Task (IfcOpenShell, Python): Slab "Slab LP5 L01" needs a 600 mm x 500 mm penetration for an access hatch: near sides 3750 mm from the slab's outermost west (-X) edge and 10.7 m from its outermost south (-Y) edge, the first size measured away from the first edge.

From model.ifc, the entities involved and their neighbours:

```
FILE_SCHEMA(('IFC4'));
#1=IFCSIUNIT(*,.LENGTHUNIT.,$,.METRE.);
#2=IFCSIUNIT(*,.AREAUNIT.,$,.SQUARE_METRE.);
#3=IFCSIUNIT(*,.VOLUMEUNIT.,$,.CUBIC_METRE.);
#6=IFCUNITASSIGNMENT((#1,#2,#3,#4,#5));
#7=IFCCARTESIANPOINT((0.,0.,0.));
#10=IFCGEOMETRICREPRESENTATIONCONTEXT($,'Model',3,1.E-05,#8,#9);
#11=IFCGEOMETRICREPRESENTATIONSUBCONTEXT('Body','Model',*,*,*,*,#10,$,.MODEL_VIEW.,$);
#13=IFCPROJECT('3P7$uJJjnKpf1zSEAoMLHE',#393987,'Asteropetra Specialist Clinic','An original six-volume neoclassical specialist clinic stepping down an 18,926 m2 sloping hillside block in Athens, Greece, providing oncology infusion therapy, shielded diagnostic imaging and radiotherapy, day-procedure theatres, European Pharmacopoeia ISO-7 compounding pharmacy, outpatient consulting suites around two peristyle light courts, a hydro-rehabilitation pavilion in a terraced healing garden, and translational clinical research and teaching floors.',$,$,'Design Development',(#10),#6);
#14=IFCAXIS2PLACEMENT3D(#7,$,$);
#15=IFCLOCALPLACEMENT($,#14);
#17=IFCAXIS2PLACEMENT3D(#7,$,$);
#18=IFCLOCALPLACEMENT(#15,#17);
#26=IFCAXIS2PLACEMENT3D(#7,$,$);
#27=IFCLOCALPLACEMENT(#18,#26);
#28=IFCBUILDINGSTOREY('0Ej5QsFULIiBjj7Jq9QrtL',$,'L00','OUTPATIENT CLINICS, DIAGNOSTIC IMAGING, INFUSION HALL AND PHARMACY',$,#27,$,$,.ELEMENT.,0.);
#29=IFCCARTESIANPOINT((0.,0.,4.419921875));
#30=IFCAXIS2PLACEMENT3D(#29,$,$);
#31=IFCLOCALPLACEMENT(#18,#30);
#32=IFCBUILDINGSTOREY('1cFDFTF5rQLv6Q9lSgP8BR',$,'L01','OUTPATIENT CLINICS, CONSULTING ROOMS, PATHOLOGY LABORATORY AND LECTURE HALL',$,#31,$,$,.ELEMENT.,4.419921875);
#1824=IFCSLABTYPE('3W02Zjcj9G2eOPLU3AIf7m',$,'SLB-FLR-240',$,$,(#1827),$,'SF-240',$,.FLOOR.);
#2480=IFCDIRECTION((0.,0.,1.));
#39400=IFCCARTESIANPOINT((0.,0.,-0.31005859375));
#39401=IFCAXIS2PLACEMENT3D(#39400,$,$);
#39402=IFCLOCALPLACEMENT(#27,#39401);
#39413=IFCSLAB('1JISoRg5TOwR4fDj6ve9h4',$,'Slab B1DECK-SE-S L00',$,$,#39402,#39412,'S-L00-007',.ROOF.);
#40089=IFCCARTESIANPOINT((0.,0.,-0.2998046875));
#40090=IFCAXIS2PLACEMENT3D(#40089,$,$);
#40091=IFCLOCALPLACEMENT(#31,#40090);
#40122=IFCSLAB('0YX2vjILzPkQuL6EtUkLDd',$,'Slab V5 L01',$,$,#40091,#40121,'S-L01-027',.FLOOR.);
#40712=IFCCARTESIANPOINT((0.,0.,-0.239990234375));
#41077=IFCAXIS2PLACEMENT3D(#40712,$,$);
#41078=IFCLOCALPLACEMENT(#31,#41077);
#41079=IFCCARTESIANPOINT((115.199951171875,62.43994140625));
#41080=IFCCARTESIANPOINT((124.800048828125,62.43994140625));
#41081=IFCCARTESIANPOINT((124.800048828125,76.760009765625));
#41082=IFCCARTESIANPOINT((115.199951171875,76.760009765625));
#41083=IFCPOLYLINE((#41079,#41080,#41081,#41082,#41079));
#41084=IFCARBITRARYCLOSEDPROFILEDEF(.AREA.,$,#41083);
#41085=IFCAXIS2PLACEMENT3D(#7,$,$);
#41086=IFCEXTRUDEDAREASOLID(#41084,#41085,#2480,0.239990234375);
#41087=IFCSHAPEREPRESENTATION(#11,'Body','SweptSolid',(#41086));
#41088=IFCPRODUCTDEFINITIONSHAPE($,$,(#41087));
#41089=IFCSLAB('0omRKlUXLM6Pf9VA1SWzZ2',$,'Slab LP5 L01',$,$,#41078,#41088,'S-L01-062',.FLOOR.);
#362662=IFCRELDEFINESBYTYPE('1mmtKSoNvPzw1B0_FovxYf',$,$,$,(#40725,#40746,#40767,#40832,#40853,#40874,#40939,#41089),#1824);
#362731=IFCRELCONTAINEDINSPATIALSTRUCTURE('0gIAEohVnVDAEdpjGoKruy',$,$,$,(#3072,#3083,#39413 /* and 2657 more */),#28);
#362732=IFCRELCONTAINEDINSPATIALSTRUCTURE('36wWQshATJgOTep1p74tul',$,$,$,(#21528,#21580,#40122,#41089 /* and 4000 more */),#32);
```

```python
import numpy as np
import ifcopenshell
import ifcopenshell.api.feature
import ifcopenshell.api.geometry
import ifcopenshell.api.root
import ifcopenshell.geom
import ifcopenshell.util.placement
import ifcopenshell.util.representation
import ifcopenshell.util.shape
import ifcopenshell.util.unit

model = ifcopenshell.open("model.ifc")
unit_scale = ifcopenshell.util.unit.calculate_unit_scale(model)
settings = ifcopenshell.geom.settings()


def volume(element):
    """Net volume in cubic metres, openings subtracted."""
    shape = ifcopenshell.geom.create_shape(settings, element)
    return ifcopenshell.util.shape.get_volume(shape.geometry)


slab = model.by_guid("0omRKlUXLM6Pf9VA1SWzZ2")
before = volume(slab)

# Extent in the slab's own axes, in metres. The edges named are its -X and -Y sides.
slab_shape = ifcopenshell.geom.create_shape(settings, slab)
vertices = ifcopenshell.util.shape.get_vertices(slab_shape.geometry)
x_min, y_min, bottom = vertices.min(axis=0)
top = vertices[:, 2].max()

opening = ifcopenshell.api.root.create_entity(model, ifc_class="IfcOpeningElement", name="Access hatch opening", predefined_type="OPENING")
context = ifcopenshell.util.representation.get_context(model, "Model", "Body", "MODEL_VIEW")
width, depth = 0.6, 0.5
outline = [(0.0, 0.0), (width, 0.0), (width, depth), (0.0, depth), (0.0, 0.0)]
# Overshoot both faces by 50 mm so the cut is clean.
shape = ifcopenshell.api.geometry.add_slab_representation(
    model, context=context, depth=top - bottom + 0.1, polyline=outline
)
ifcopenshell.api.geometry.assign_representation(model, product=opening, representation=shape)

matrix = ifcopenshell.util.placement.get_local_placement(slab.ObjectPlacement)
matrix[:, 3] = matrix @ np.append(np.array([x_min + 3.75, y_min + 10.7, bottom - 0.05]) / unit_scale, 1.0)
ifcopenshell.api.geometry.edit_object_placement(model, product=opening, matrix=matrix, is_si=False)
ifcopenshell.api.feature.add_feature(model, feature=opening, element=slab)

after = volume(slab)

print(f"slab volume {before:.3f} -> {after:.3f} m3")

model.write("model_updated.ifc")
```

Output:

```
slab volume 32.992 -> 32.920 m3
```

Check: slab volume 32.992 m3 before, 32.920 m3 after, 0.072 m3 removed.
